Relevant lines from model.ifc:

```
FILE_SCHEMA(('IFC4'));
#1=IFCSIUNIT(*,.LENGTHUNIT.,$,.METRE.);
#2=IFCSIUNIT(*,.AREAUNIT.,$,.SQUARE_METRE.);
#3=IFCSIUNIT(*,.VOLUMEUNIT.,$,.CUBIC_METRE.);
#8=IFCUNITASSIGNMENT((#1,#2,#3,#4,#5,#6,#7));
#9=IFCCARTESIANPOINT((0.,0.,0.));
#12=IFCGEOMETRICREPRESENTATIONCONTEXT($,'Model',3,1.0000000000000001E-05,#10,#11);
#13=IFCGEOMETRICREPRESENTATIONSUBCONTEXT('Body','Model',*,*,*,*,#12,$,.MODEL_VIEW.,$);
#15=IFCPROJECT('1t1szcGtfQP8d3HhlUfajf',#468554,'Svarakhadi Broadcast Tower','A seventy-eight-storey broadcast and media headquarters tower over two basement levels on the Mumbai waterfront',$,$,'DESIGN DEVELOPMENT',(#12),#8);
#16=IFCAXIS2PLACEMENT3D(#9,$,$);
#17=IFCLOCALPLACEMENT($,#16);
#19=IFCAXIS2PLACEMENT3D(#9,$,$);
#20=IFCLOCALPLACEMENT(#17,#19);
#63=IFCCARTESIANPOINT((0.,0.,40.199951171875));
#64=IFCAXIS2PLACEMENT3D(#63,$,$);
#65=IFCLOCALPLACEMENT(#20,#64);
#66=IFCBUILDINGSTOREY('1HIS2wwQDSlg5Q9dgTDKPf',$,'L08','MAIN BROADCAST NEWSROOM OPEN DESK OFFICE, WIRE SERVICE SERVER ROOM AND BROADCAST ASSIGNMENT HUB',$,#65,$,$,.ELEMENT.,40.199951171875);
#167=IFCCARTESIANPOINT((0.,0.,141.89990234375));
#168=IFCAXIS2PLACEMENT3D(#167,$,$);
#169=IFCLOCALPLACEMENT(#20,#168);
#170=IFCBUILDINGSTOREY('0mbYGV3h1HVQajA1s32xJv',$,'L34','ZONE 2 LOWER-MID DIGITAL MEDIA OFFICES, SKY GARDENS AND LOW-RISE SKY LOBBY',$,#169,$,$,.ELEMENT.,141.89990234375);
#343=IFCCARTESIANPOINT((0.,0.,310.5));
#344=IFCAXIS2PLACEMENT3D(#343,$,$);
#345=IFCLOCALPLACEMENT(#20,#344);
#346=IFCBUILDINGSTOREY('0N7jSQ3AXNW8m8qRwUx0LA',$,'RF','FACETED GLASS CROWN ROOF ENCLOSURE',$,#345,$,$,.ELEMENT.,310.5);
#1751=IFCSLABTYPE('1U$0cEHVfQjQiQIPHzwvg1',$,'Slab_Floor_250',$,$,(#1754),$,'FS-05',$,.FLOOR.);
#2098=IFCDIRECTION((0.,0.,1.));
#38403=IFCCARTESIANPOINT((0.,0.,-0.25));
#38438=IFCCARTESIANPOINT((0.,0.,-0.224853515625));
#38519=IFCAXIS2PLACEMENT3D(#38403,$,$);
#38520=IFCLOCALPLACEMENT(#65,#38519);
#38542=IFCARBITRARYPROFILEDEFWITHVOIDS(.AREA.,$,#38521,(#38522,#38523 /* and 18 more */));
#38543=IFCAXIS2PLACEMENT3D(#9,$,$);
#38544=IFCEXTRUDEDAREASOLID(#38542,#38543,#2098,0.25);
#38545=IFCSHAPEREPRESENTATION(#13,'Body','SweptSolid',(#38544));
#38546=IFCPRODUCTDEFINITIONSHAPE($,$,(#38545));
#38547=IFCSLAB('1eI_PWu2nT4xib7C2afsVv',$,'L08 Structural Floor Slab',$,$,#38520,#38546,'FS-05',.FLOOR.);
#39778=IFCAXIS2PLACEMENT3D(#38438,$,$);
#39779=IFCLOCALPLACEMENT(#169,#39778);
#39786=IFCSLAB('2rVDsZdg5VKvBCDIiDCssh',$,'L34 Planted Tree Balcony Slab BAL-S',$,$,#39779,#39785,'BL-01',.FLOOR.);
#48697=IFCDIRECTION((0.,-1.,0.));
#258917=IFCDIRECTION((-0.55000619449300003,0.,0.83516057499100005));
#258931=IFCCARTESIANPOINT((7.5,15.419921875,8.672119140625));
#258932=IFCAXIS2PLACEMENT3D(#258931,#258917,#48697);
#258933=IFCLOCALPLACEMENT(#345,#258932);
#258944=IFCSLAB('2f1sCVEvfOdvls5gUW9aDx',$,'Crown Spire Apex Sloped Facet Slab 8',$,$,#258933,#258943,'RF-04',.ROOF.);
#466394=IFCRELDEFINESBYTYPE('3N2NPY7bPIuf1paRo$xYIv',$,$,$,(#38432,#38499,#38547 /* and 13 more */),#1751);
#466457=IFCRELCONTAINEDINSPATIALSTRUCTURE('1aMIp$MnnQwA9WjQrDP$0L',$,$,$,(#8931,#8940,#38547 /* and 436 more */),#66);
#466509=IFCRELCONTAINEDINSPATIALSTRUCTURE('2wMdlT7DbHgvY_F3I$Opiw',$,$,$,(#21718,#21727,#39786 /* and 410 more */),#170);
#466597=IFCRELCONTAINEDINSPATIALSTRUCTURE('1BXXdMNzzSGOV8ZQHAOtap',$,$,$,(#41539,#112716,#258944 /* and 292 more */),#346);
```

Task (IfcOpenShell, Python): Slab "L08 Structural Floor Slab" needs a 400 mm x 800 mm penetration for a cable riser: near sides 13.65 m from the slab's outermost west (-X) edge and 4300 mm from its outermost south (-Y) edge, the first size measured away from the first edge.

```python
import numpy as np
import ifcopenshell
import ifcopenshell.api.feature
import ifcopenshell.api.geometry
import ifcopenshell.api.root
import ifcopenshell.geom
import ifcopenshell.util.placement
import ifcopenshell.util.representation
import ifcopenshell.util.shape
import ifcopenshell.util.unit

model = ifcopenshell.open("model.ifc")
unit_scale = ifcopenshell.util.unit.calculate_unit_scale(model)
settings = ifcopenshell.geom.settings()


def volume(element):
    """Net volume in cubic metres, openings subtracted."""
    shape = ifcopenshell.geom.create_shape(settings, element)
    return ifcopenshell.util.shape.get_volume(shape.geometry)


slab = model.by_guid("1eI_PWu2nT4xib7C2afsVv")
before = volume(slab)

# Extent in the slab's own axes, in metres. The edges named are its -X and -Y sides.
slab_shape = ifcopenshell.geom.create_shape(settings, slab)
vertices = ifcopenshell.util.shape.get_vertices(slab_shape.geometry)
x_min, y_min, bottom = vertices.min(axis=0)
top = vertices[:, 2].max()

opening = ifcopenshell.api.root.create_entity(model, ifc_class="IfcOpeningElement", name="Cable riser opening", predefined_type="OPENING")
context = ifcopenshell.util.representation.get_context(model, "Model", "Body", "MODEL_VIEW")
width, depth = 0.4, 0.8
outline = [(0.0, 0.0), (width, 0.0), (width, depth), (0.0, depth), (0.0, 0.0)]
# Overshoot both faces by 50 mm so the cut is clean.
shape = ifcopenshell.api.geometry.add_slab_representation(
    model, context=context, depth=top - bottom + 0.1, polyline=outline
)
ifcopenshell.api.geometry.assign_representation(model, product=opening, representation=shape)

matrix = ifcopenshell.util.placement.get_local_placement(slab.ObjectPlacement)
matrix[:, 3] = matrix @ np.append(np.array([x_min + 13.65, y_min + 4.3, bottom - 0.05]) / unit_scale, 1.0)
ifcopenshell.api.geometry.edit_object_placement(model, product=opening, matrix=matrix, is_si=False)
ifcopenshell.api.feature.add_feature(model, feature=opening, element=slab)

after = volume(slab)

print(f"slab volume {before:.3f} -> {after:.3f} m3")

model.write("model-out.ifc")
```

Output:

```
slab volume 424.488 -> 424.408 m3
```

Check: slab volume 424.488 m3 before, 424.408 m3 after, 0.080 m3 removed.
